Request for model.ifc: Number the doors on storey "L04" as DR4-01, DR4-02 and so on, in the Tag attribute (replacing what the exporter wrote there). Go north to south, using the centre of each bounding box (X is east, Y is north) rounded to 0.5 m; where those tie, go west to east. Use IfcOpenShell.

First a look at what the model holds.

```python
import ifcopenshell
import ifcopenshell.util.element
import ifcopenshell.util.placement

model = ifcopenshell.open("model.ifc")
print(model.schema)
storey = next(s for s in model.by_type("IfcBuildingStorey") if s.Name == "L04")
doors = [e for e in ifcopenshell.util.element.get_decomposition(storey) if e.is_a("IfcDoor")]
for e in sorted(doors, key=lambda e: e.id()):
    origin = ifcopenshell.util.placement.get_local_placement(e.ObjectPlacement)[:3, 3]
    print(e.id(), e.Tag, e.Name, origin.round(2) + 0.0, sep=" | ")
```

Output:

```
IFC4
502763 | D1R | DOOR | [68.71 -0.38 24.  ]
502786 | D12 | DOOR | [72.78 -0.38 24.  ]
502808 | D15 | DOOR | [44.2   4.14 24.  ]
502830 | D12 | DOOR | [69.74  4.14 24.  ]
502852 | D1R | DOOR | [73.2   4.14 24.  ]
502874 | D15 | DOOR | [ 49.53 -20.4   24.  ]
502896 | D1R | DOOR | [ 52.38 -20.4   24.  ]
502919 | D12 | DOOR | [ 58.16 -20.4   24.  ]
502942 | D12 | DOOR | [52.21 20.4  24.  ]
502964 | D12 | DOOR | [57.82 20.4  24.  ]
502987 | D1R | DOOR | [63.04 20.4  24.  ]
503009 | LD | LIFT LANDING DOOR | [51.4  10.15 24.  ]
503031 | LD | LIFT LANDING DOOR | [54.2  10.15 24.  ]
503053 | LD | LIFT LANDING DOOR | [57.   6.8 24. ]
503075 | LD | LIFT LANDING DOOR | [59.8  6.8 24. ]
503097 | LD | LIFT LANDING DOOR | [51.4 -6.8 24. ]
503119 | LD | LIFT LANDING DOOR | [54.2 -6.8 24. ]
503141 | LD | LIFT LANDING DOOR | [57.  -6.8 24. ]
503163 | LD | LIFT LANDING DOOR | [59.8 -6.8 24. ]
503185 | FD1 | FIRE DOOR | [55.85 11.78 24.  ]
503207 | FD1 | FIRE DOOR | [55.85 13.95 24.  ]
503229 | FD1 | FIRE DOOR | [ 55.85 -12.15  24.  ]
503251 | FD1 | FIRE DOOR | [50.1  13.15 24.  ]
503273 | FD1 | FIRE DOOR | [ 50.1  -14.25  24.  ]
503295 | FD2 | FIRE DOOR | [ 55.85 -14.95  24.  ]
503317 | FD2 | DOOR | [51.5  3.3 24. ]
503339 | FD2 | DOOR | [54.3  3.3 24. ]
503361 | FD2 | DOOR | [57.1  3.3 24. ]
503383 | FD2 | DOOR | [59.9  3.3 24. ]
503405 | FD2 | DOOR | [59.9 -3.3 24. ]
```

```python
import ifcopenshell
import ifcopenshell.geom
import ifcopenshell.util.element
import ifcopenshell.util.shape

model = ifcopenshell.open("model.ifc")
settings = ifcopenshell.geom.settings()
settings.set("use-world-coords", True)


def centre(element):
    shape = ifcopenshell.geom.create_shape(settings, element)
    return ifcopenshell.util.shape.get_bbox_centroid(shape.geometry)


storey = next(s for s in model.by_type("IfcBuildingStorey") if s.Name == "L04")
doors = [e for e in ifcopenshell.util.element.get_decomposition(storey) if e.is_a("IfcDoor")]

# Insertion points can sit at a corner or the storey origin, so sort by the geometry (in metres).
centres = {e: centre(e) for e in doors}
doors.sort(key=lambda e: (-round(centres[e][1] / 0.5), centres[e][0]))

for i, e in enumerate(doors, start=1):
    number = f"DR4-{i:02d}"
    e.Tag = number
    print(e.id(), number)

model.write("model-out.ifc")
```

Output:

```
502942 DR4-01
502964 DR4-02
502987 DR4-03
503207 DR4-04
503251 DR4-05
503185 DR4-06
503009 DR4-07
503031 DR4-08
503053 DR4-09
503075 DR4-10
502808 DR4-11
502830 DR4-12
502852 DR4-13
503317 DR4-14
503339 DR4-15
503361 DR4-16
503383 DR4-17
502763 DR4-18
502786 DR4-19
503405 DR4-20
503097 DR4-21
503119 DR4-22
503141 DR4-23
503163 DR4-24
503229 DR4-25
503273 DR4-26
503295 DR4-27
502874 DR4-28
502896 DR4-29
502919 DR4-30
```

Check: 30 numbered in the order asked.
